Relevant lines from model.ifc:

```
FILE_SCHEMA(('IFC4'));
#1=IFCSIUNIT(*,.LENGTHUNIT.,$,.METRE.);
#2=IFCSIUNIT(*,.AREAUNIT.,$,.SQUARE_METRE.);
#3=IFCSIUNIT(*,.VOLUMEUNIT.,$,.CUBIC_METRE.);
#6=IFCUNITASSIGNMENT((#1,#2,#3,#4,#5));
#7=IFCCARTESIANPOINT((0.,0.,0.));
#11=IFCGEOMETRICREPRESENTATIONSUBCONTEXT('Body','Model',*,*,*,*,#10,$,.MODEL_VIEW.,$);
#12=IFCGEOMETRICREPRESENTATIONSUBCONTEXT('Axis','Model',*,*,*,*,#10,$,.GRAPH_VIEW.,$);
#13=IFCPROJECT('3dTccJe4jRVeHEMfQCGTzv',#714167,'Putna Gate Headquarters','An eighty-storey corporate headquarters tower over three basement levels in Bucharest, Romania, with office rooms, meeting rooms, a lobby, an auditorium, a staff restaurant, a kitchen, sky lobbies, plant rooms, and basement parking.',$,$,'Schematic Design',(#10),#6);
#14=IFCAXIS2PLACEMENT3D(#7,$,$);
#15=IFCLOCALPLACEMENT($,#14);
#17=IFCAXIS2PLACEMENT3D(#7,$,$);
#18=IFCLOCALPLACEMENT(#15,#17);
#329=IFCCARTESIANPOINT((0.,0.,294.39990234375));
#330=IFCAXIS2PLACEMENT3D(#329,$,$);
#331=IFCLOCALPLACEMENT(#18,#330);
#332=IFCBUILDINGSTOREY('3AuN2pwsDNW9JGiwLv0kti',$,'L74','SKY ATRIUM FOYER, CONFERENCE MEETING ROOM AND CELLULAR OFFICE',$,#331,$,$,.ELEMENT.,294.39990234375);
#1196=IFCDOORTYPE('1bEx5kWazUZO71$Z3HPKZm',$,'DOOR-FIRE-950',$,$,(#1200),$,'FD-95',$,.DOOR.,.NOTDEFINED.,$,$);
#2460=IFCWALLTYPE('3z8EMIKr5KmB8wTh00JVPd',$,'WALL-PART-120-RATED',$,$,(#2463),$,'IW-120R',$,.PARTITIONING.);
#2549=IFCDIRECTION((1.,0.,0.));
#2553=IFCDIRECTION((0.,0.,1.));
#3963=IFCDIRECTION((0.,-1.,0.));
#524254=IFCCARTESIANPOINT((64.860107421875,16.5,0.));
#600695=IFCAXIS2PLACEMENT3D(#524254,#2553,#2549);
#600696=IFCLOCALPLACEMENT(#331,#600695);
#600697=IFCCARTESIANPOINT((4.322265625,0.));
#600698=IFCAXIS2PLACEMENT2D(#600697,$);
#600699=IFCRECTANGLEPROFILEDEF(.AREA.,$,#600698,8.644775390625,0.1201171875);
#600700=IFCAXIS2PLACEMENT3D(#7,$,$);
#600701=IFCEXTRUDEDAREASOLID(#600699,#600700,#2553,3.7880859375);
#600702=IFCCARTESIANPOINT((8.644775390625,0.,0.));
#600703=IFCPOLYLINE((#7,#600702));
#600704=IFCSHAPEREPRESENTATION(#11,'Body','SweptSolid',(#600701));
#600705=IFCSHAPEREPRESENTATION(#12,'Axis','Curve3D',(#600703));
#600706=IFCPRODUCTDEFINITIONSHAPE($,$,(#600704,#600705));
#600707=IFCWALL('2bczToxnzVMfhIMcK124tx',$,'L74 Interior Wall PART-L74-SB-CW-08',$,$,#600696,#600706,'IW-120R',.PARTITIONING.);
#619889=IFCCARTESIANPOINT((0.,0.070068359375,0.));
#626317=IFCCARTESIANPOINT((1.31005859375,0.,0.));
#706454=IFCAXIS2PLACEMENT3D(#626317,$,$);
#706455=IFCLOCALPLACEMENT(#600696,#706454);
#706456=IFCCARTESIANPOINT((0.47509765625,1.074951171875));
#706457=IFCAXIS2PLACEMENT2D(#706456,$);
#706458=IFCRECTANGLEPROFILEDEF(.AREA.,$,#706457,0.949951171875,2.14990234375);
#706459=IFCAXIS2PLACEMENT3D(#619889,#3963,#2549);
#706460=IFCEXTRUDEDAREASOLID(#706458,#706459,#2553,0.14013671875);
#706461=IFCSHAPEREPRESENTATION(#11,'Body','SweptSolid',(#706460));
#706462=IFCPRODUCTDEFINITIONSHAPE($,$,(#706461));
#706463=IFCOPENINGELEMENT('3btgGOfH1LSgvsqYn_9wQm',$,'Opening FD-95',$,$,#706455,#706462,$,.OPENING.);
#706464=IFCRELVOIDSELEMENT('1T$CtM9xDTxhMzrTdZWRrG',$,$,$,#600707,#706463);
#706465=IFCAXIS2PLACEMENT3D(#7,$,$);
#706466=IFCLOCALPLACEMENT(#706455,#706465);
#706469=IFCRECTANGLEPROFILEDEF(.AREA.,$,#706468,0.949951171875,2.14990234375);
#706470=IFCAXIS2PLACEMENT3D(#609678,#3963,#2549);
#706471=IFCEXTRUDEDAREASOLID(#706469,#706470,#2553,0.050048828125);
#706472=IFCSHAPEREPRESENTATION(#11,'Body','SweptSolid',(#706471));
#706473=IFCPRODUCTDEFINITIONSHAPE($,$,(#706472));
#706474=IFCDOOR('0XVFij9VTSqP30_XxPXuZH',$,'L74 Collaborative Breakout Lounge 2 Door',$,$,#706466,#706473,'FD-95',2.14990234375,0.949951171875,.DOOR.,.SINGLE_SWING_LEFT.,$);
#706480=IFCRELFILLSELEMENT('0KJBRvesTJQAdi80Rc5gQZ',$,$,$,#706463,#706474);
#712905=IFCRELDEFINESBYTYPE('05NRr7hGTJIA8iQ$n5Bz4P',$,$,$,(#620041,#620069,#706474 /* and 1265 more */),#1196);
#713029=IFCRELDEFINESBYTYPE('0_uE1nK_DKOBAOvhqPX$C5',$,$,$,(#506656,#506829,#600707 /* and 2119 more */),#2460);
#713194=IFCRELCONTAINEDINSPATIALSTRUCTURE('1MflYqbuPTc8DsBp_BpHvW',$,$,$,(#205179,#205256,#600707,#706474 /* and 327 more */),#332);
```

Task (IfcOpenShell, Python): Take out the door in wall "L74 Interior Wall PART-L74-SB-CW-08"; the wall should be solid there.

```python
import ifcopenshell
import ifcopenshell.api.feature
import ifcopenshell.api.root
import ifcopenshell.geom
import ifcopenshell.util.shape

model = ifcopenshell.open("model.ifc")
settings = ifcopenshell.geom.settings()


def volume(element):
    """Net volume in cubic metres, openings subtracted."""
    shape = ifcopenshell.geom.create_shape(settings, element)
    return ifcopenshell.util.shape.get_volume(shape.geometry)


door = model.by_guid("0XVFij9VTSqP30_XxPXuZH")
opening = door.FillsVoids[0].RelatingOpeningElement
wall = opening.VoidsElements[0].RelatingBuildingElement
before = volume(wall)

ifcopenshell.api.root.remove_product(model, product=door)
ifcopenshell.api.feature.remove_feature(model, feature=opening)

after = volume(wall)

print(f"wall volume {before:.3f} -> {after:.3f} m3")

model.write("model-out.ifc")
```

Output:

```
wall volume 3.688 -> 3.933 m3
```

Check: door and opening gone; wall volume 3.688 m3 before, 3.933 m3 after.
